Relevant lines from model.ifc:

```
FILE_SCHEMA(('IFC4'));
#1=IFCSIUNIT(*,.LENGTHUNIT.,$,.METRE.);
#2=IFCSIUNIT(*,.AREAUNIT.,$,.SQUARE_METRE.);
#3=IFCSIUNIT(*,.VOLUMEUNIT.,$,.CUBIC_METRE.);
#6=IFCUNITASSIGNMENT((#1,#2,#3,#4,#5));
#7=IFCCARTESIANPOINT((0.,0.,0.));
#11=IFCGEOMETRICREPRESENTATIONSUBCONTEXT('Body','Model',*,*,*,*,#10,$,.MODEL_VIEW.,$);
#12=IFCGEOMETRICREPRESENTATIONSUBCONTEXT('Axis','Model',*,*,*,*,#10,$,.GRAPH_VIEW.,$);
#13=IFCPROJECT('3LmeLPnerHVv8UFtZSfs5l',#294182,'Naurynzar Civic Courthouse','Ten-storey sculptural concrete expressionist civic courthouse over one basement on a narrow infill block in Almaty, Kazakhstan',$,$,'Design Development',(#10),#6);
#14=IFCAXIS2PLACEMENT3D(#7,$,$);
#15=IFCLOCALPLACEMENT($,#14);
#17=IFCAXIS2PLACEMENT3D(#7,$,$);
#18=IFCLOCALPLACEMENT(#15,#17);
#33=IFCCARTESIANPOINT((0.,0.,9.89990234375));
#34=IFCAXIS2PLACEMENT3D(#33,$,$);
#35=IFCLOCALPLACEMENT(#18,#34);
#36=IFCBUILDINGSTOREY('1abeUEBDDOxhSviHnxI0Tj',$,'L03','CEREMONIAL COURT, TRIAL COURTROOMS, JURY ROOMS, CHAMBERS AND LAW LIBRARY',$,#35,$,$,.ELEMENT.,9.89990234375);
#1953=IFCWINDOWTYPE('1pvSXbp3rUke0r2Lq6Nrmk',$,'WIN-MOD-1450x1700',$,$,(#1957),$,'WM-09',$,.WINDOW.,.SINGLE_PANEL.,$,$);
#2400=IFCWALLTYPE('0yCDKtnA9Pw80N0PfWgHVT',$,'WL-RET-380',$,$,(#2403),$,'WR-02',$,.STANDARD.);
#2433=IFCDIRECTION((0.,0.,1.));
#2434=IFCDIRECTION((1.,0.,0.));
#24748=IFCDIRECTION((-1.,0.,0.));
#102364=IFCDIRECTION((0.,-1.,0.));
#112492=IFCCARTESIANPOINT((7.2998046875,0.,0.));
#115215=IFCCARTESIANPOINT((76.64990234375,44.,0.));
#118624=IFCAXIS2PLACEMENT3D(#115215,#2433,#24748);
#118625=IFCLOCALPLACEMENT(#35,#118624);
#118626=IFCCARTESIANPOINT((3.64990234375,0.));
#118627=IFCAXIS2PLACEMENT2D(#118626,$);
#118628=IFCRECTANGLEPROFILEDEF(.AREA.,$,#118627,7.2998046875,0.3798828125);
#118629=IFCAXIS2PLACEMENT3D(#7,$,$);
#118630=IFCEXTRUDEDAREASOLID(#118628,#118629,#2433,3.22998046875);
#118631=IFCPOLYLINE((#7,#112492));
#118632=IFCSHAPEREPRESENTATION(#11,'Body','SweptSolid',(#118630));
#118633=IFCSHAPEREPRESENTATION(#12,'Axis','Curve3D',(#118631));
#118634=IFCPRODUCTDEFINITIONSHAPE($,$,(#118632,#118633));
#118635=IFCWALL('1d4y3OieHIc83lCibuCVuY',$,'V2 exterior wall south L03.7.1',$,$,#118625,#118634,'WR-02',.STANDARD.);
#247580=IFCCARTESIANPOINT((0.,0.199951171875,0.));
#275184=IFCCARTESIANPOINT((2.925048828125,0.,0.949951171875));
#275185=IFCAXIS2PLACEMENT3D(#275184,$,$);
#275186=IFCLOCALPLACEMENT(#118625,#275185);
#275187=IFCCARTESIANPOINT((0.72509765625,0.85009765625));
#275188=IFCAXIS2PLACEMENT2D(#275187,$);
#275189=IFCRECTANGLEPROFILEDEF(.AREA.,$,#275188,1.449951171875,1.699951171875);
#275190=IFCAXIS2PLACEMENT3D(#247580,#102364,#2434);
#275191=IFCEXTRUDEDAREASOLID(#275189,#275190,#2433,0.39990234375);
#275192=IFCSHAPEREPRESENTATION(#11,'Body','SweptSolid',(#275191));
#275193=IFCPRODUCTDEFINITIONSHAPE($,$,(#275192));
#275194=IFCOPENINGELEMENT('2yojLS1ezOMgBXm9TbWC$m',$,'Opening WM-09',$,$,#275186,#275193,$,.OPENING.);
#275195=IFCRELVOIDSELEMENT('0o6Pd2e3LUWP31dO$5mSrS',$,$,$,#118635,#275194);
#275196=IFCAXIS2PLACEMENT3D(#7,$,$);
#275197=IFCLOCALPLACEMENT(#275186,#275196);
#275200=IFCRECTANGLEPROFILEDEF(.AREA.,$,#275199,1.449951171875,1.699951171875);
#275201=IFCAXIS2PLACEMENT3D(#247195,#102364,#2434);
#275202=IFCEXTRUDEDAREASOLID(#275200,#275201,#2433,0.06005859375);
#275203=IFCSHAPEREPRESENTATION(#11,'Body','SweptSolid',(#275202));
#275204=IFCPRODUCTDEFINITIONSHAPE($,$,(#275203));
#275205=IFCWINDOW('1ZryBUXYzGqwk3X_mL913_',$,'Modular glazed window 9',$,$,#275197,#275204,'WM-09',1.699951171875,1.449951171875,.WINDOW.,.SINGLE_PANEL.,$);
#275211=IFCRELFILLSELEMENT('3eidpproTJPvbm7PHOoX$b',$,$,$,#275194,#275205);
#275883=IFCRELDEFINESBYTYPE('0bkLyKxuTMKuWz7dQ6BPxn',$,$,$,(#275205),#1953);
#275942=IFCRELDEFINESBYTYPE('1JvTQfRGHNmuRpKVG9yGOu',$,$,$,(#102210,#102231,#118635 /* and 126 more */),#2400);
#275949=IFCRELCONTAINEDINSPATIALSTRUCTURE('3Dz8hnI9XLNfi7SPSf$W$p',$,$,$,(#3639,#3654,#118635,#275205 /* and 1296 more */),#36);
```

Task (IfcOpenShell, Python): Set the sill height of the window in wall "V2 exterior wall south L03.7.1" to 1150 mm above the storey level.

```python
import numpy as np
import ifcopenshell
import ifcopenshell.api.geometry
import ifcopenshell.geom
import ifcopenshell.util.element
import ifcopenshell.util.placement
import ifcopenshell.util.shape
import ifcopenshell.util.unit

model = ifcopenshell.open("model.ifc")
unit_scale = ifcopenshell.util.unit.calculate_unit_scale(model)

window = model.by_guid("1ZryBUXYzGqwk3X_mL913_")
opening = window.FillsVoids[0].RelatingOpeningElement
storey = ifcopenshell.util.element.get_container(window, ifc_class="IfcBuildingStorey")
level = ifcopenshell.util.placement.get_local_placement(storey.ObjectPlacement)[2, 3]

# The opening's origin need not be at the sill, so measure its lowest point.
shape = ifcopenshell.geom.create_shape(ifcopenshell.geom.settings(), opening)
bottom = ifcopenshell.util.shape.get_shape_bottom_elevation(shape, shape.geometry) / unit_scale
dz = level + 1.15 / unit_scale - bottom

shift = np.array([0.0, 0.0, dz])
# The window is placed relative to its opening, so it follows when the opening moves.
matrix = ifcopenshell.util.placement.get_local_placement(opening.ObjectPlacement)
matrix[:3, 3] += shift
ifcopenshell.api.geometry.edit_object_placement(
    model, product=opening, matrix=matrix, is_si=False, should_transform_children=True
)

print(f"moved by {dz * unit_scale:+.3f} m")

model.write("model-out.ifc")
```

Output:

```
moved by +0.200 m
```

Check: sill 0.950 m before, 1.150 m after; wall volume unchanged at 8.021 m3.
